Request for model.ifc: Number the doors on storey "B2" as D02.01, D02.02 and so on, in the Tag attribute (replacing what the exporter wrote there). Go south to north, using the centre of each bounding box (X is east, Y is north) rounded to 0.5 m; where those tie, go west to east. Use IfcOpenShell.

First a look at what the model holds.

```python
import ifcopenshell
import ifcopenshell.util.element
import ifcopenshell.util.placement

model = ifcopenshell.open("model.ifc")
print(model.schema)
storey = next(s for s in model.by_type("IfcBuildingStorey") if s.Name == "B2")
doors = [e for e in ifcopenshell.util.element.get_decomposition(storey) if e.is_a("IfcDoor")]
for e in sorted(doors, key=lambda e: e.id()):
    origin = ifcopenshell.util.placement.get_local_placement(e.ObjectPlacement)[:3, 3]
    print(e.id(), e.Tag, e.Name, origin.round(2) + 0.0, sep=" | ")
```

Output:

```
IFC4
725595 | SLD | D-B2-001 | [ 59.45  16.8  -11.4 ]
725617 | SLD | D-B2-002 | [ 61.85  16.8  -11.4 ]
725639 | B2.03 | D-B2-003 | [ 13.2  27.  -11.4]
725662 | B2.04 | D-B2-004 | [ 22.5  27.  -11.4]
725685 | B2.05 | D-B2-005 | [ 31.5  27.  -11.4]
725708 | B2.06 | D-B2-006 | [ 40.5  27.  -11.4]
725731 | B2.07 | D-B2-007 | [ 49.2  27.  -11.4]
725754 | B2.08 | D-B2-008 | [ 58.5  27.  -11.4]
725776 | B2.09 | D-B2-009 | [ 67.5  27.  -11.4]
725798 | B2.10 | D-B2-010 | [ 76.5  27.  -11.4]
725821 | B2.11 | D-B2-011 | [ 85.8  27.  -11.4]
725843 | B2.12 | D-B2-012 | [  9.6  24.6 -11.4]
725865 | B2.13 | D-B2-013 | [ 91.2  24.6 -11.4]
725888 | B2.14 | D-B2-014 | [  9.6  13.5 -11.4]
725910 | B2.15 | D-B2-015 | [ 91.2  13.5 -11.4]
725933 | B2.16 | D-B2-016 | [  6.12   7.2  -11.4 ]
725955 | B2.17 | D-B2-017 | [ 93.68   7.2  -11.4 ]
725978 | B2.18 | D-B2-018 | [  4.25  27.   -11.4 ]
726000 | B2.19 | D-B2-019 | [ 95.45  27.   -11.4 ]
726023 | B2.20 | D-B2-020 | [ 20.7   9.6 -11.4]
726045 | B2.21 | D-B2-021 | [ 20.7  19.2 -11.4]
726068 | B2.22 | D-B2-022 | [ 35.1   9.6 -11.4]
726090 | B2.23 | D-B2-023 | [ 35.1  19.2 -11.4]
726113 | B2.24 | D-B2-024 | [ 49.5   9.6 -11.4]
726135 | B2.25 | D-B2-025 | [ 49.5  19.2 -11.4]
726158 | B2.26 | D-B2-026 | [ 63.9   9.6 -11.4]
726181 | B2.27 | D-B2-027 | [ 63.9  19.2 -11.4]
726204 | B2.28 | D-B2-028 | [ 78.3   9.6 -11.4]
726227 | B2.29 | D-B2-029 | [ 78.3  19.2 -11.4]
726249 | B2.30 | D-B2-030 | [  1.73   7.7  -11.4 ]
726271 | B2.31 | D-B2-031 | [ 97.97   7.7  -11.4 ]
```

```python
import ifcopenshell
import ifcopenshell.geom
import ifcopenshell.util.element
import ifcopenshell.util.shape

model = ifcopenshell.open("model.ifc")
settings = ifcopenshell.geom.settings()
settings.set("use-world-coords", True)


def centre(element):
    shape = ifcopenshell.geom.create_shape(settings, element)
    return ifcopenshell.util.shape.get_bbox_centroid(shape.geometry)


storey = next(s for s in model.by_type("IfcBuildingStorey") if s.Name == "B2")
doors = [e for e in ifcopenshell.util.element.get_decomposition(storey) if e.is_a("IfcDoor")]

# Insertion points can sit at a corner or the storey origin, so sort by the geometry (in metres).
centres = {e: centre(e) for e in doors}
doors.sort(key=lambda e: (round(centres[e][1] / 0.5), centres[e][0]))

for i, e in enumerate(doors, start=1):
    number = f"D02.{i:02d}"
    e.Tag = number
    print(e.id(), number)

model.write("model-out.ifc")
```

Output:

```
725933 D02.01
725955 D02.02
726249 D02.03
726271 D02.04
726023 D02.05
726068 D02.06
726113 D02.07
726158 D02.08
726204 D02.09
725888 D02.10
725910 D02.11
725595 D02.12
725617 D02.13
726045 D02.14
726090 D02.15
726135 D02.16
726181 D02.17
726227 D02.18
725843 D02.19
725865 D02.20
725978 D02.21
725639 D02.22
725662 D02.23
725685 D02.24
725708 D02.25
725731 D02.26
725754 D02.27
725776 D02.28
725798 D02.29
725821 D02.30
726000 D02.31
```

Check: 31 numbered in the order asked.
